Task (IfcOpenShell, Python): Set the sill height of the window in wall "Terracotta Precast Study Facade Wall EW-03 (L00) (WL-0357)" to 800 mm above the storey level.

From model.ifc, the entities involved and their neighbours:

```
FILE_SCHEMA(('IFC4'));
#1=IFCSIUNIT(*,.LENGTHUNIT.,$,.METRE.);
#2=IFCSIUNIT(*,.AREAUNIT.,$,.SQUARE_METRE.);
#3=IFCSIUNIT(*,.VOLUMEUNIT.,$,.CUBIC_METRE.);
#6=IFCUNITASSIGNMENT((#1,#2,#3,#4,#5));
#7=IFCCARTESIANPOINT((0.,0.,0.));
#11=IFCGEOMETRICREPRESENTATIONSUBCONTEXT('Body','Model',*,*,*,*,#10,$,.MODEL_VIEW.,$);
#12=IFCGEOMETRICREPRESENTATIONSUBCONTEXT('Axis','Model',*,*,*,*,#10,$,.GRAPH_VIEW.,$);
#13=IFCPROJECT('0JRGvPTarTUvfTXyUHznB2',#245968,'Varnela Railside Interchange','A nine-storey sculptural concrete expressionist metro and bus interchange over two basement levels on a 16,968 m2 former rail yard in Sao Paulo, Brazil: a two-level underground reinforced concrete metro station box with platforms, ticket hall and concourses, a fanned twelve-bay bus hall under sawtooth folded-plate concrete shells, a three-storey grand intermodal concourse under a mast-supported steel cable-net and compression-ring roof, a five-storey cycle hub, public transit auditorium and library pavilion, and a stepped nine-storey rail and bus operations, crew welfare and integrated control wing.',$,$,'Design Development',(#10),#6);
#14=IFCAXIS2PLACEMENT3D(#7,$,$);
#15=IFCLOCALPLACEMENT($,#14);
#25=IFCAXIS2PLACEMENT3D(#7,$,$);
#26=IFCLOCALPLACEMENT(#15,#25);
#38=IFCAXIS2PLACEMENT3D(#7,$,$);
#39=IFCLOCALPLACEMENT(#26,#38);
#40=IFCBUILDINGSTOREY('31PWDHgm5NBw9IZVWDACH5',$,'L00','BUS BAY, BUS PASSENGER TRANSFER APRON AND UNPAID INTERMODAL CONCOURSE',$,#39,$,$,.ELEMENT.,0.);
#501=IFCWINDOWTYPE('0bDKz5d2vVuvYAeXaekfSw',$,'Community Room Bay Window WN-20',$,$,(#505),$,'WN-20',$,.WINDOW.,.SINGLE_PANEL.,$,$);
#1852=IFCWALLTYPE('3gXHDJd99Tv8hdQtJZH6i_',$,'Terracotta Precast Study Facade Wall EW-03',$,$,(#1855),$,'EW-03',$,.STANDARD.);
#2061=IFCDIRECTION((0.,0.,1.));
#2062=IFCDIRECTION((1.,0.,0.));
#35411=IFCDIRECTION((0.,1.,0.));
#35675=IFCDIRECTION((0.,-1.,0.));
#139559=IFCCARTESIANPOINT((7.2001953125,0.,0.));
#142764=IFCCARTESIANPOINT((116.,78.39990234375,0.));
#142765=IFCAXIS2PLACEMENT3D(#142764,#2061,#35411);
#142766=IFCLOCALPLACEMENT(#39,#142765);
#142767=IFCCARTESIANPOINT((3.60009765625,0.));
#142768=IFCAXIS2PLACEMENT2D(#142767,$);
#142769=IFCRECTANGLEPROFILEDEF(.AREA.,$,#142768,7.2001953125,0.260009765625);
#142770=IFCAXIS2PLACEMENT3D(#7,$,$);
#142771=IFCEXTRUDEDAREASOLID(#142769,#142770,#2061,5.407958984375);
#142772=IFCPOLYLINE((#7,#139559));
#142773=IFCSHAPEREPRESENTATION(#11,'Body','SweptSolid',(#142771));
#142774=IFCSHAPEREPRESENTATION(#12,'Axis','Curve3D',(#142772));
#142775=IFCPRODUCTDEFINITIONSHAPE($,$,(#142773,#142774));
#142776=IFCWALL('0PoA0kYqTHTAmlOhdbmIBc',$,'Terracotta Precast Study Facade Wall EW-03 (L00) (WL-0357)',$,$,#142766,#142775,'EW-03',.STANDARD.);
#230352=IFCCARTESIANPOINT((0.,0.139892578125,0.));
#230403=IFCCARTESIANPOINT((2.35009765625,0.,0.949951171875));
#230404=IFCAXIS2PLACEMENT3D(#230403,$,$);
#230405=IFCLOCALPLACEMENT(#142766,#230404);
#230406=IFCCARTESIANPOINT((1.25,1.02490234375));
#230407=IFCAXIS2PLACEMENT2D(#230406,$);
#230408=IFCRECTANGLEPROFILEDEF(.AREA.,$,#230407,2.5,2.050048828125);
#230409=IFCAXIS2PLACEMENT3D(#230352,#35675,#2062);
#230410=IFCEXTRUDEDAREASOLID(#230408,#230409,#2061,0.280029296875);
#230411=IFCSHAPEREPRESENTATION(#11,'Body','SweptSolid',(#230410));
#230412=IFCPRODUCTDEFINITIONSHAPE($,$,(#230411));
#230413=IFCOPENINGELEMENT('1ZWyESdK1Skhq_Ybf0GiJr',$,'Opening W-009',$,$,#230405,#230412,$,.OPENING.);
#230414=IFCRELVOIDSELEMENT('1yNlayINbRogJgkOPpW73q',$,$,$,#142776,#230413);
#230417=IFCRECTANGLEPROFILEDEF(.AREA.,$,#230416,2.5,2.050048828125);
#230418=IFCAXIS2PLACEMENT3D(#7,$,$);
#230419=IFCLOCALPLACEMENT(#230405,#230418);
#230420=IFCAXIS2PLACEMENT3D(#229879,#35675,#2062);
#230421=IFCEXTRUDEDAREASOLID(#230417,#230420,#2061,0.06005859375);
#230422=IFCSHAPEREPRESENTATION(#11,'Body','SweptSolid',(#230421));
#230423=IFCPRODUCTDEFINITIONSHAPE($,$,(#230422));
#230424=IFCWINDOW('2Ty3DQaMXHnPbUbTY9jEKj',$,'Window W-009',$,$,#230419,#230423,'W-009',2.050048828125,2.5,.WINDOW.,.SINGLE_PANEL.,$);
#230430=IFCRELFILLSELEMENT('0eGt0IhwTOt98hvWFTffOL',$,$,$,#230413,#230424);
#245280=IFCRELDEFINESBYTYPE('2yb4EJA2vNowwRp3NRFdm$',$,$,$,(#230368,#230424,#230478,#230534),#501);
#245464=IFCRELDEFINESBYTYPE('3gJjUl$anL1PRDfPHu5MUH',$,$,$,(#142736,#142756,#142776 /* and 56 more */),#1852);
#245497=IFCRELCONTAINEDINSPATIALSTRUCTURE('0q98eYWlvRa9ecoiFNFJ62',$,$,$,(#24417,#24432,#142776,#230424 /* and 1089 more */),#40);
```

```python
import numpy as np
import ifcopenshell
import ifcopenshell.api.geometry
import ifcopenshell.geom
import ifcopenshell.util.element
import ifcopenshell.util.placement
import ifcopenshell.util.shape
import ifcopenshell.util.unit

model = ifcopenshell.open("model.ifc")
unit_scale = ifcopenshell.util.unit.calculate_unit_scale(model)

window = model.by_guid("2Ty3DQaMXHnPbUbTY9jEKj")
opening = window.FillsVoids[0].RelatingOpeningElement
storey = ifcopenshell.util.element.get_container(window, ifc_class="IfcBuildingStorey")
level = ifcopenshell.util.placement.get_local_placement(storey.ObjectPlacement)[2, 3]

# The opening's origin need not be at the sill, so measure its lowest point.
shape = ifcopenshell.geom.create_shape(ifcopenshell.geom.settings(), opening)
bottom = ifcopenshell.util.shape.get_shape_bottom_elevation(shape, shape.geometry) / unit_scale
dz = level + 0.8 - bottom

shift = np.array([0.0, 0.0, dz])
# The window is placed relative to its opening, so it follows when the opening moves.
matrix = ifcopenshell.util.placement.get_local_placement(opening.ObjectPlacement)
matrix[:3, 3] += shift
ifcopenshell.api.geometry.edit_object_placement(
    model, product=opening, matrix=matrix, is_si=False, should_transform_children=True
)

print(f"moved by {dz * unit_scale:+.3f} m")

model.write("model_rev.ifc")
```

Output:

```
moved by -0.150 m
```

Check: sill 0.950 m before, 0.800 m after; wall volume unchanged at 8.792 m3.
